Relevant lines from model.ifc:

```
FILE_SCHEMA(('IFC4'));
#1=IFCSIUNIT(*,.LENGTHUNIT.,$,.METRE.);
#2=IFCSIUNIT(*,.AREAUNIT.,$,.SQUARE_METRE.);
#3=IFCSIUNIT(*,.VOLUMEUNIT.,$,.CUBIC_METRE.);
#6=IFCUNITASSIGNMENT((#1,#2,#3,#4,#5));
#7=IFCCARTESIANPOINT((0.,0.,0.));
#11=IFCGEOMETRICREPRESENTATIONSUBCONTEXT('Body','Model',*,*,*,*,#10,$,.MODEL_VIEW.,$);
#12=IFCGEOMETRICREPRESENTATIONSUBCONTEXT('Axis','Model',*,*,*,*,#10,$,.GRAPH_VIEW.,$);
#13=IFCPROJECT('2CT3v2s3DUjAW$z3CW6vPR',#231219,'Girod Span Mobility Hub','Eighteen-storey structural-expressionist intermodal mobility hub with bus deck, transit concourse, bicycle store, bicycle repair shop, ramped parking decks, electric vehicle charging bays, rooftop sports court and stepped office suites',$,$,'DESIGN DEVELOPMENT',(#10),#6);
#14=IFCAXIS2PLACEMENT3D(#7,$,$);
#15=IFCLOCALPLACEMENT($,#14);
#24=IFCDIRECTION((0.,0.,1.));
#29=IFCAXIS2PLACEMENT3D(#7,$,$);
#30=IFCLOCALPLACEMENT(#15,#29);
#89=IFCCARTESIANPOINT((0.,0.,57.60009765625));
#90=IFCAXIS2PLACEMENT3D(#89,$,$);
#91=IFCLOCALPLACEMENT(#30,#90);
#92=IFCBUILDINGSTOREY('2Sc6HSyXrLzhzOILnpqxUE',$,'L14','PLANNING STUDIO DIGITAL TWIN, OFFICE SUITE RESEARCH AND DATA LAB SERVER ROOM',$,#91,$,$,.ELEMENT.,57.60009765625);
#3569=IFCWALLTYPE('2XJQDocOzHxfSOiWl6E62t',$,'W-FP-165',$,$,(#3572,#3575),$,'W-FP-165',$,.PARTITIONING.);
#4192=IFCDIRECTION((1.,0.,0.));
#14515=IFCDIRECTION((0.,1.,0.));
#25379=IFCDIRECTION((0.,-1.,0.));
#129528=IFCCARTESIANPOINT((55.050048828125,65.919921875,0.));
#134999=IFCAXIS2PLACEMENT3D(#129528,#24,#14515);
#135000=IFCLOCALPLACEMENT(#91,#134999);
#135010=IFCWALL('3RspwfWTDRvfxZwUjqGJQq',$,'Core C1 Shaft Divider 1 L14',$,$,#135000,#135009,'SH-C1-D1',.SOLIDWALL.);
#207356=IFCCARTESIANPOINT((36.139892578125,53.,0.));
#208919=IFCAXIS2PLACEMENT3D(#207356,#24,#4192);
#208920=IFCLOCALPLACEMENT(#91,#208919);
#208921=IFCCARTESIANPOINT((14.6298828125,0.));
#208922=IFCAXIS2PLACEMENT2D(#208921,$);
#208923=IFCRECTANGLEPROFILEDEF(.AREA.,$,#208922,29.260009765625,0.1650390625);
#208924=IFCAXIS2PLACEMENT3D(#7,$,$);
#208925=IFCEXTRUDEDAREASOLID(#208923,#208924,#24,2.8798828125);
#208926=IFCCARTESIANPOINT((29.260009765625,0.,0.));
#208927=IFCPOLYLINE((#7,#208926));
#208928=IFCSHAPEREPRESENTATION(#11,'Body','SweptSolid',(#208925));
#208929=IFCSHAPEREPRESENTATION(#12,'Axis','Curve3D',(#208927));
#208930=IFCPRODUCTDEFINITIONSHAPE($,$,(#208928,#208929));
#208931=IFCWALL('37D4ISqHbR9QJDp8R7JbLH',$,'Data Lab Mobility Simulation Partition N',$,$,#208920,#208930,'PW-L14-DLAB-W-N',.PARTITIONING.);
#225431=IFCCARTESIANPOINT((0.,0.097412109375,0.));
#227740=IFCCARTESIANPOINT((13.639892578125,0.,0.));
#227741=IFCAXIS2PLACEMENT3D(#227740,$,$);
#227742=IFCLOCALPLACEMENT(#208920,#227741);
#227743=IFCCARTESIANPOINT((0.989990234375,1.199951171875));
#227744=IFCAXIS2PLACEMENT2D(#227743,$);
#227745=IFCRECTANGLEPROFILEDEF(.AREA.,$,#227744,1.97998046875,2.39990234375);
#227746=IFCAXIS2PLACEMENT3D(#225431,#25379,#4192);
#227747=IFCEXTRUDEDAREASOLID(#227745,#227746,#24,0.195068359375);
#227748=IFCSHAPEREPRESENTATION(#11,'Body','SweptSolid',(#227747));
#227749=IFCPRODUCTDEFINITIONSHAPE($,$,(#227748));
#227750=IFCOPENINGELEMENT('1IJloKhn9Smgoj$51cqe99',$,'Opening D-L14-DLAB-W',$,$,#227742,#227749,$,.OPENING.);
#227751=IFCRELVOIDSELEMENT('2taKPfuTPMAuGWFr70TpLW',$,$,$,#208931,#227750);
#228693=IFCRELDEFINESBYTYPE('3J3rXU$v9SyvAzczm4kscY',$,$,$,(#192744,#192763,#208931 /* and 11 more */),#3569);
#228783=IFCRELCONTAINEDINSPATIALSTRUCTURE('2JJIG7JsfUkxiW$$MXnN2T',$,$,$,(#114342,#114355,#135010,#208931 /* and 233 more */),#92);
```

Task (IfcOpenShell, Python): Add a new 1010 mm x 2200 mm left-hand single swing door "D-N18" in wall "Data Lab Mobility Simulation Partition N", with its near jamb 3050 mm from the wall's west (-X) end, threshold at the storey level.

```python
import numpy as np
import ifcopenshell
import ifcopenshell.api.feature
import ifcopenshell.api.geometry
import ifcopenshell.api.root
import ifcopenshell.api.spatial
import ifcopenshell.geom
import ifcopenshell.util.element
import ifcopenshell.util.placement
import ifcopenshell.util.representation
import ifcopenshell.util.shape
import ifcopenshell.util.unit

model = ifcopenshell.open("model.ifc")
unit_scale = ifcopenshell.util.unit.calculate_unit_scale(model)
settings = ifcopenshell.geom.settings()


def volume(element):
    """Net volume in cubic metres, openings subtracted."""
    shape = ifcopenshell.geom.create_shape(settings, element)
    return ifcopenshell.util.shape.get_volume(shape.geometry)


wall = model.by_id(208931)
storey = ifcopenshell.util.element.get_container(wall, ifc_class="IfcBuildingStorey")
context = ifcopenshell.util.representation.get_context(model, "Model", "Body", "MODEL_VIEW")
before = volume(wall)

width, height, from_end, sill = 1.01, 2.2, 3.05, 0.0  # metres

# The wall runs along its own X axis, and the end named is its -X end.
wall_shape = ifcopenshell.geom.create_shape(settings, wall)
x, y, z = ifcopenshell.util.shape.get_vertices(wall_shape.geometry).T
start = x.min() + from_end
face, thickness = float(y.min()), float(y.max() - y.min())
wall_matrix = ifcopenshell.util.placement.get_local_placement(wall.ObjectPlacement)
level = ifcopenshell.util.placement.get_local_placement(storey.ObjectPlacement)[2, 3]


def in_wall(x, y):
    """Placement at x, y metres in the wall's axes, at sill height."""
    matrix = wall_matrix.copy()
    matrix[:, 3] = wall_matrix @ np.array([x / unit_scale, y / unit_scale, 0.0, 1.0])
    matrix[2, 3] = level + sill / unit_scale
    return matrix


# Opening: a box that overshoots both wall faces by 50 mm.
opening = ifcopenshell.api.root.create_entity(model, ifc_class="IfcOpeningElement", predefined_type="OPENING")
box = ifcopenshell.api.geometry.add_wall_representation(
    model, context=context, length=width, height=height, thickness=thickness + 0.1
)
ifcopenshell.api.geometry.assign_representation(model, product=opening, representation=box)
ifcopenshell.api.geometry.edit_object_placement(model, product=opening, matrix=in_wall(start, face - 0.05), is_si=False)
ifcopenshell.api.feature.add_feature(model, feature=opening, element=wall)

door = ifcopenshell.api.root.create_entity(model, ifc_class="IfcDoor", name="D-N18", predefined_type="DOOR")
door.OverallWidth, door.OverallHeight = width / unit_scale, height / unit_scale
door.OperationType = "SINGLE_SWING_LEFT"
body = ifcopenshell.api.geometry.add_door_representation(
    model,
    context=context,
    overall_width=door.OverallWidth,
    overall_height=door.OverallHeight,
    operation_type="SINGLE_SWING_LEFT",
    lining_properties={"LiningDepth": thickness / unit_scale, "ThresholdDepth": thickness / unit_scale},
)
ifcopenshell.api.geometry.assign_representation(model, product=door, representation=body)
ifcopenshell.api.spatial.assign_container(model, products=[door], relating_structure=storey)
ifcopenshell.api.feature.add_filling(model, opening=opening, element=door)

# The lining spans the wall, so the door starts at the wall face.
ifcopenshell.api.geometry.edit_object_placement(model, product=door, matrix=in_wall(start, face), is_si=False)

after = volume(wall)

print(f"wall volume {before:.3f} -> {after:.3f} m3")

model.write("model-out.ifc")
```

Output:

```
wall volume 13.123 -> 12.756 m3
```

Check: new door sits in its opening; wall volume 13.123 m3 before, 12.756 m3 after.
